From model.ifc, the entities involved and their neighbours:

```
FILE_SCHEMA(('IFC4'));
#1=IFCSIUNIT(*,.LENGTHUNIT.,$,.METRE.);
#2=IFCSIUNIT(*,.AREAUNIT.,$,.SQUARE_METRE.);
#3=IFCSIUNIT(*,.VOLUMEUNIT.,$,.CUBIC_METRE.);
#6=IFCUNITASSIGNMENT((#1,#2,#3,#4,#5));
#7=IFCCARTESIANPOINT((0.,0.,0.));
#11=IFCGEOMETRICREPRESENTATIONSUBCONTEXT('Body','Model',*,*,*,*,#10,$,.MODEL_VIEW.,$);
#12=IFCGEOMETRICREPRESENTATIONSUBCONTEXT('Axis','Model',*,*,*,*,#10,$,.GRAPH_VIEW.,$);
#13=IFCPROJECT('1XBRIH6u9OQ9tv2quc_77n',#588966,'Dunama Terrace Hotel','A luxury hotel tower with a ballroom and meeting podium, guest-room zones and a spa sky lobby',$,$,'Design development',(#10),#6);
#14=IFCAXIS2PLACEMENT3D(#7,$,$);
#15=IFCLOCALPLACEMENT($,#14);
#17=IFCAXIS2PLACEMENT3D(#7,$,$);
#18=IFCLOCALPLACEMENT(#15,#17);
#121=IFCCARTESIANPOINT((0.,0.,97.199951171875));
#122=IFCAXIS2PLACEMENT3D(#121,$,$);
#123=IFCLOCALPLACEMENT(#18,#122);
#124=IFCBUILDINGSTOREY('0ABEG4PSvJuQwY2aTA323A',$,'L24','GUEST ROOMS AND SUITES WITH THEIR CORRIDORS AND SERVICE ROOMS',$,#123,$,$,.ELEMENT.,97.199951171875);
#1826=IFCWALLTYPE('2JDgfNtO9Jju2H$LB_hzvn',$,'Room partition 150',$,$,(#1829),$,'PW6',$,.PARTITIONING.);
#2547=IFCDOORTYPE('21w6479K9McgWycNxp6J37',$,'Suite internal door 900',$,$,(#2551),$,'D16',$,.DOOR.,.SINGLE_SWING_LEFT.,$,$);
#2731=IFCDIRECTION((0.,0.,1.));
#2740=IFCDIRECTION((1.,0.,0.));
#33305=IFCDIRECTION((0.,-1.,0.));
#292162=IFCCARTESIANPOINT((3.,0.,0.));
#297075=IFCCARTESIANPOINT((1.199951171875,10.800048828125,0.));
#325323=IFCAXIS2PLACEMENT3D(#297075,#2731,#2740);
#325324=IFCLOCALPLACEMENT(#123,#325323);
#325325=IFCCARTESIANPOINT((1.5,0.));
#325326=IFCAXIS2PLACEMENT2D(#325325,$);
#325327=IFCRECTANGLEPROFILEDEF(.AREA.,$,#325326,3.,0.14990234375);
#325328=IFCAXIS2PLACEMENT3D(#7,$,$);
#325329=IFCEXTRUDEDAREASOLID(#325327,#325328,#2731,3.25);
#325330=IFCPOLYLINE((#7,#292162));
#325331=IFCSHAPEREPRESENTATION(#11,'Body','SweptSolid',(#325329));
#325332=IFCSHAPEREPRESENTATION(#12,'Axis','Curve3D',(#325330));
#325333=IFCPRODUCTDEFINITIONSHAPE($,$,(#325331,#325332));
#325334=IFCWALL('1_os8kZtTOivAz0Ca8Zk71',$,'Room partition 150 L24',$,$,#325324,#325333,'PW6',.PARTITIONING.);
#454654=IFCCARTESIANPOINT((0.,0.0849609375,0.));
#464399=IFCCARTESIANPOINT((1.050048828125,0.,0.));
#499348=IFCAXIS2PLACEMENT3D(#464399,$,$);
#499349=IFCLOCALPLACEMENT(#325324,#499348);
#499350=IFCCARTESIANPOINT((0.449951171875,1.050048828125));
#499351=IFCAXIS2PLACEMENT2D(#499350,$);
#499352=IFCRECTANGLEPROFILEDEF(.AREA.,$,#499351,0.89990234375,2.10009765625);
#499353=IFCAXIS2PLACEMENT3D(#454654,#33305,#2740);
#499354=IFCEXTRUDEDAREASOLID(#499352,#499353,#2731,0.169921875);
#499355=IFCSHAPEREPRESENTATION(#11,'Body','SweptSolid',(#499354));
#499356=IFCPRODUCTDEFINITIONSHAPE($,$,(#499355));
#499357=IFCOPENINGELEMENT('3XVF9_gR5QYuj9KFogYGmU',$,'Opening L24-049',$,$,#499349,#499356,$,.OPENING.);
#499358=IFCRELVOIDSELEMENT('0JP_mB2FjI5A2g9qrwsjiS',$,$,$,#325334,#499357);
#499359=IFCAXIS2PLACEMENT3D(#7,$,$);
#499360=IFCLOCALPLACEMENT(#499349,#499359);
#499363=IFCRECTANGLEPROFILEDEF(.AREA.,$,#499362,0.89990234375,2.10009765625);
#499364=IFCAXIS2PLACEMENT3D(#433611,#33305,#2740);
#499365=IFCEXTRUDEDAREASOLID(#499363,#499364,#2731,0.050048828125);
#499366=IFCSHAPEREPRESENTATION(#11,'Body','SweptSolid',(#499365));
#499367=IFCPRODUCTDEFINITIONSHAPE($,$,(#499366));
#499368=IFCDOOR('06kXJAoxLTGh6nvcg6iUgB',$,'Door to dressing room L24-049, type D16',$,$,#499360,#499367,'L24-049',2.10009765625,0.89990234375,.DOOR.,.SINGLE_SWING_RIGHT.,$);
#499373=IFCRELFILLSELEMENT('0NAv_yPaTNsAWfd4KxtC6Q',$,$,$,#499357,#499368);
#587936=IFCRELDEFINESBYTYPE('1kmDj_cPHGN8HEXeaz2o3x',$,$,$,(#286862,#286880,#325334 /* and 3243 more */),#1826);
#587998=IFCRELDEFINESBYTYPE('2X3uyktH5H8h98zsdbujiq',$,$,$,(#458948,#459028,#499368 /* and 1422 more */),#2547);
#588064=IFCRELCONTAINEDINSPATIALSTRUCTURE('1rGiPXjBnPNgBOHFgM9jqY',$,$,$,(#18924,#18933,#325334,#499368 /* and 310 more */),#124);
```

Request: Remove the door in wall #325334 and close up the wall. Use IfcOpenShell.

```python
import ifcopenshell
import ifcopenshell.api.feature
import ifcopenshell.api.root
import ifcopenshell.geom
import ifcopenshell.util.shape

model = ifcopenshell.open("model.ifc")
settings = ifcopenshell.geom.settings()


def volume(element):
    """Net volume in cubic metres, openings subtracted."""
    shape = ifcopenshell.geom.create_shape(settings, element)
    return ifcopenshell.util.shape.get_volume(shape.geometry)


door = model.by_guid("06kXJAoxLTGh6nvcg6iUgB")
opening = door.FillsVoids[0].RelatingOpeningElement
wall = opening.VoidsElements[0].RelatingBuildingElement
before = volume(wall)

ifcopenshell.api.root.remove_product(model, product=door)
ifcopenshell.api.feature.remove_feature(model, feature=opening)

after = volume(wall)

print(f"wall volume {before:.3f} -> {after:.3f} m3")

model.write("model_edited.ifc")
```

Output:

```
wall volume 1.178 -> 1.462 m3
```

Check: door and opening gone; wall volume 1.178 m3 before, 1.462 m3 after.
